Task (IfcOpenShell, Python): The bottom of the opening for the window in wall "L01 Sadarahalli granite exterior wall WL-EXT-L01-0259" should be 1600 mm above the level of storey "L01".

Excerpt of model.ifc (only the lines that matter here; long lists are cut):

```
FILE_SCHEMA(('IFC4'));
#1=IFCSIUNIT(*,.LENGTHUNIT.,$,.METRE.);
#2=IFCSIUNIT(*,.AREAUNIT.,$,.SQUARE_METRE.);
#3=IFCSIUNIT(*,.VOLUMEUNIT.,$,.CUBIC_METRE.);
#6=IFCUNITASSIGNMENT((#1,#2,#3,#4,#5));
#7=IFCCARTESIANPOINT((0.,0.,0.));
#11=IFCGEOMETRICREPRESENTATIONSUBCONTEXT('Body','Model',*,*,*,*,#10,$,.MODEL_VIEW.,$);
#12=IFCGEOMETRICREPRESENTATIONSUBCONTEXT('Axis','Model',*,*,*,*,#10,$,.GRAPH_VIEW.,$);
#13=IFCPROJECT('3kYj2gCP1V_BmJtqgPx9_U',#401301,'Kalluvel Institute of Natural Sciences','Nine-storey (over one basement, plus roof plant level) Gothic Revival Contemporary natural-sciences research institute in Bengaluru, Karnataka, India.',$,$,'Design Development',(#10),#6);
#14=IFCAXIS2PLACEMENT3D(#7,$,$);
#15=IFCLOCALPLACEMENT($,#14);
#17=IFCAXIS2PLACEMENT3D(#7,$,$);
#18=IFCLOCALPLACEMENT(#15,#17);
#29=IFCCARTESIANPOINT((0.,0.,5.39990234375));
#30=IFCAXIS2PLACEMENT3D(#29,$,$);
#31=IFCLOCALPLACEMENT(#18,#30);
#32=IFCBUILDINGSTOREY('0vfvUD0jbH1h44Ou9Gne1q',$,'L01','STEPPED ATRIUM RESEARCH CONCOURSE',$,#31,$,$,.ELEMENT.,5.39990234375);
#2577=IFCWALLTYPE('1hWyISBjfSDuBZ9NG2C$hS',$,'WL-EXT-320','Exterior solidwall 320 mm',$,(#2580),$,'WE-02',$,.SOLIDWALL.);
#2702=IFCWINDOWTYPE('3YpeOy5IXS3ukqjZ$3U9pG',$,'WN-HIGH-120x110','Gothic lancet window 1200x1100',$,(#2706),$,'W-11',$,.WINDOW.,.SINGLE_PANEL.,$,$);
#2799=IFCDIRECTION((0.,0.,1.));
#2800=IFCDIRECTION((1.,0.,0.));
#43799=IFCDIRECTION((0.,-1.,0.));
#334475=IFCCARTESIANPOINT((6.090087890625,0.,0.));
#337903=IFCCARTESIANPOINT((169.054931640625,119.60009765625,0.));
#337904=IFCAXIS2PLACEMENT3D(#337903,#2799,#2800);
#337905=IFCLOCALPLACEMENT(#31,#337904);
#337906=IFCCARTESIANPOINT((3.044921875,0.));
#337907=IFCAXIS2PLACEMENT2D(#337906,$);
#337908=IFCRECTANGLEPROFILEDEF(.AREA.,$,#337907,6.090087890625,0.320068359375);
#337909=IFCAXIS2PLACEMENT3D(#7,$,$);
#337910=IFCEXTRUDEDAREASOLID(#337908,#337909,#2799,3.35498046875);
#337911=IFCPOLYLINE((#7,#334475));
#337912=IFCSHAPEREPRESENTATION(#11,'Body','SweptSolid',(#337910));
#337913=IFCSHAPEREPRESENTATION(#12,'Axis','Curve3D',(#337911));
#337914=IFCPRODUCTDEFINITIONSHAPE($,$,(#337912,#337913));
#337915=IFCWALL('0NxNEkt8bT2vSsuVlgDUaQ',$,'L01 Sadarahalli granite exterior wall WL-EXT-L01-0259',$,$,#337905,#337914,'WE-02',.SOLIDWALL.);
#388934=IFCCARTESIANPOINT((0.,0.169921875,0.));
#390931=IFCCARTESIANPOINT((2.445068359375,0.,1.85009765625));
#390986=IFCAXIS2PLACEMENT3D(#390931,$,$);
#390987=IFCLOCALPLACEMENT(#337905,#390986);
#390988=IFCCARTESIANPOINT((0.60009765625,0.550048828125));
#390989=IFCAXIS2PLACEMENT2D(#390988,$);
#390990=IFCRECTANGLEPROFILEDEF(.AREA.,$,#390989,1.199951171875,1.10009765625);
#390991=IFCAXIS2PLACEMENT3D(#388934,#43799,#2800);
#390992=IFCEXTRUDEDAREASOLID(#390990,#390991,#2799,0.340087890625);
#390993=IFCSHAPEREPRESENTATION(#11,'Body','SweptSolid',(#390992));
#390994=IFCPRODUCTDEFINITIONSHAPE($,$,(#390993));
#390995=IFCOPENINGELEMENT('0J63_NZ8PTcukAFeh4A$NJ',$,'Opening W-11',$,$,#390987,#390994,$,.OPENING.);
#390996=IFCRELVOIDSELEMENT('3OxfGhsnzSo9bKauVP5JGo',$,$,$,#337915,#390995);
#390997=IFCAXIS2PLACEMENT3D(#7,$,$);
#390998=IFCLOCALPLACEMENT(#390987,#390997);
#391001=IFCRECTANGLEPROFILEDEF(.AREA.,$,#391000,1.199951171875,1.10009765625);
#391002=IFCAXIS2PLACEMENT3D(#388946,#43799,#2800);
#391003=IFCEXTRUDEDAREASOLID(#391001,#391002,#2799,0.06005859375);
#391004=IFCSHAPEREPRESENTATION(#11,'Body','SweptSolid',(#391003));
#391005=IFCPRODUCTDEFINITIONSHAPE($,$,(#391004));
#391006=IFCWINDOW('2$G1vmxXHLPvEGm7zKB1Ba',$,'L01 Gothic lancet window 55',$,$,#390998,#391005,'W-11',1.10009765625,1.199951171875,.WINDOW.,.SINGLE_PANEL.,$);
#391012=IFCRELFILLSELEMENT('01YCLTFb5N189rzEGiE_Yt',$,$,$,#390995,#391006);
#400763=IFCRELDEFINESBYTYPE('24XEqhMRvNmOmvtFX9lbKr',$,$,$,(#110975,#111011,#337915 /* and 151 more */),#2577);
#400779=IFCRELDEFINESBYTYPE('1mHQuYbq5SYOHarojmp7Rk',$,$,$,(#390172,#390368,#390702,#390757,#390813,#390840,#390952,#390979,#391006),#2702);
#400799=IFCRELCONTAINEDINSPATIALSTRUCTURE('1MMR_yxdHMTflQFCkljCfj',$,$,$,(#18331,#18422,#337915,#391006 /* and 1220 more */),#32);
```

```python
import numpy as np
import ifcopenshell
import ifcopenshell.api.geometry
import ifcopenshell.geom
import ifcopenshell.util.element
import ifcopenshell.util.placement
import ifcopenshell.util.shape
import ifcopenshell.util.unit

model = ifcopenshell.open("model.ifc")
unit_scale = ifcopenshell.util.unit.calculate_unit_scale(model)

window = model.by_guid("2$G1vmxXHLPvEGm7zKB1Ba")
opening = window.FillsVoids[0].RelatingOpeningElement
storey = ifcopenshell.util.element.get_container(window, ifc_class="IfcBuildingStorey")
level = ifcopenshell.util.placement.get_local_placement(storey.ObjectPlacement)[2, 3]

# The opening's origin need not be at the sill, so measure its lowest point.
shape = ifcopenshell.geom.create_shape(ifcopenshell.geom.settings(), opening)
bottom = ifcopenshell.util.shape.get_shape_bottom_elevation(shape, shape.geometry) / unit_scale
dz = level + 1.6 / unit_scale - bottom

shift = np.array([0.0, 0.0, dz])
# The window is placed relative to its opening, so it follows when the opening moves.
matrix = ifcopenshell.util.placement.get_local_placement(opening.ObjectPlacement)
matrix[:3, 3] += shift
ifcopenshell.api.geometry.edit_object_placement(
    model, product=opening, matrix=matrix, is_si=False, should_transform_children=True
)

print(f"moved by {dz * unit_scale:+.3f} m")

model.write("model_v2.ifc")
```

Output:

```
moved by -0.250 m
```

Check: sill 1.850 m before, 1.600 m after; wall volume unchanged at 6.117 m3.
